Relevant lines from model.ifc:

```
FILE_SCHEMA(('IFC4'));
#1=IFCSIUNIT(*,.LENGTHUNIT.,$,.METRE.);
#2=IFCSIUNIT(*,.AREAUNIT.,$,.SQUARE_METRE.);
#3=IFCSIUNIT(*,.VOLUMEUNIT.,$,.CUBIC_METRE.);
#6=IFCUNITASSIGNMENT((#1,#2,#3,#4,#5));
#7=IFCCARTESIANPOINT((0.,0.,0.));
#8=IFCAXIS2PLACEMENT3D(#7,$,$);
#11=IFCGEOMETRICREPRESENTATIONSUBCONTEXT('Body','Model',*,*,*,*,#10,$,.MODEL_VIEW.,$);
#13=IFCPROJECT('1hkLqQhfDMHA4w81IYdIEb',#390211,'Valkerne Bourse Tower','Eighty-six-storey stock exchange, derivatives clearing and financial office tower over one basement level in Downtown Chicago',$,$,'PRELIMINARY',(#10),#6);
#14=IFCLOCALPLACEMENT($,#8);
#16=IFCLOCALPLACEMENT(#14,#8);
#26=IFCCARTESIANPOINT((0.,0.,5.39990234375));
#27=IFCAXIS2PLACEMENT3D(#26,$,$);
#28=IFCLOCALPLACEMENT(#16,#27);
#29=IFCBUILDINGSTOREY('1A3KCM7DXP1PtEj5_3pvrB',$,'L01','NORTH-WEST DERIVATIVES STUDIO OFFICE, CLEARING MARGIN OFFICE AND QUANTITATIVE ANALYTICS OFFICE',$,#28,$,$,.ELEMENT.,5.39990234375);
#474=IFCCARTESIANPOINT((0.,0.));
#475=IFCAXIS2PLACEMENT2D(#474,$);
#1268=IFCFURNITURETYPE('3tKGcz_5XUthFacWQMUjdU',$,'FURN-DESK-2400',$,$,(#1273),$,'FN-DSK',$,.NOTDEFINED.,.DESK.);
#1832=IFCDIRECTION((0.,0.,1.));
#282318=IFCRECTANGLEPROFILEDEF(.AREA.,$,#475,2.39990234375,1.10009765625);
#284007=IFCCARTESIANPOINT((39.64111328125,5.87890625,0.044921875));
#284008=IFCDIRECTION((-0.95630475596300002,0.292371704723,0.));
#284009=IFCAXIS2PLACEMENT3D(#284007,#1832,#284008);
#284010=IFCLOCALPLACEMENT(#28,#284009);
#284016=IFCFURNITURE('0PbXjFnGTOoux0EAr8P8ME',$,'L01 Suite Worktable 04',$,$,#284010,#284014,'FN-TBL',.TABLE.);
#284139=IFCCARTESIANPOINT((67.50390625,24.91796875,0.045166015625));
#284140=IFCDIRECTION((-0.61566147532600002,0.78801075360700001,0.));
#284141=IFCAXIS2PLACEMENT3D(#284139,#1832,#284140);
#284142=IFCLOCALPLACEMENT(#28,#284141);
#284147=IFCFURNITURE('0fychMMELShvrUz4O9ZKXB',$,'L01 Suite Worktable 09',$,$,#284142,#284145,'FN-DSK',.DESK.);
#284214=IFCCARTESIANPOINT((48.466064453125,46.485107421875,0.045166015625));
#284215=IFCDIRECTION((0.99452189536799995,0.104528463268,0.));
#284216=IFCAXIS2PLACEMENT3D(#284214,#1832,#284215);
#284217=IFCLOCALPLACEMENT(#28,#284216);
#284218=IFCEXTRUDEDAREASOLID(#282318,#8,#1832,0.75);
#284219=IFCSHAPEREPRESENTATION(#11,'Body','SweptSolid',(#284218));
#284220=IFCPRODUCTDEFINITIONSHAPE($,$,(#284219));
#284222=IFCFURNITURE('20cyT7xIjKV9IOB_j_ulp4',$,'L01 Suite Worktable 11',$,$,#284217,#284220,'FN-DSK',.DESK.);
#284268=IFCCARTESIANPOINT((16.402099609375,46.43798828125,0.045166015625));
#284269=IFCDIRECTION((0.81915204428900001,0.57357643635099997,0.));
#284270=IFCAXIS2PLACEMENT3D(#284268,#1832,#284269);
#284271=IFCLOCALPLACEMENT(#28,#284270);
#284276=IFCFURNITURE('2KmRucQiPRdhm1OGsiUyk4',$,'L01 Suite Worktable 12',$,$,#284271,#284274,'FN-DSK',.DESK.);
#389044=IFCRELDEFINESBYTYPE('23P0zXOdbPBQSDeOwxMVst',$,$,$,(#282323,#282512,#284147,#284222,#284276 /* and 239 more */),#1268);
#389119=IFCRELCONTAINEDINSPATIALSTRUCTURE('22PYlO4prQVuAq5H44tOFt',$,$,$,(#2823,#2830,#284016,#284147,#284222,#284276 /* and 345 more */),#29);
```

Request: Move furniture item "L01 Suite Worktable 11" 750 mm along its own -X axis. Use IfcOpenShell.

```python
import ifcopenshell
import ifcopenshell.api.geometry
import ifcopenshell.util.placement
import ifcopenshell.util.unit

model = ifcopenshell.open("model.ifc")
unit_scale = ifcopenshell.util.unit.calculate_unit_scale(model)

item = model.by_id(284222)
matrix = ifcopenshell.util.placement.get_local_placement(item.ObjectPlacement)
matrix[:3, 3] -= matrix[:3, 0] * 0.75 / unit_scale
ifcopenshell.api.geometry.edit_object_placement(model, product=item, matrix=matrix, is_si=False)

print(ifcopenshell.util.placement.get_local_placement(item.ObjectPlacement).round(3) + 0.0)

model.write("model_v2.ifc")
```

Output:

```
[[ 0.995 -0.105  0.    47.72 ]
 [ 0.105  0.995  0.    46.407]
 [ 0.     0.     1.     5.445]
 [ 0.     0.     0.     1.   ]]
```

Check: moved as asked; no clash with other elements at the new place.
